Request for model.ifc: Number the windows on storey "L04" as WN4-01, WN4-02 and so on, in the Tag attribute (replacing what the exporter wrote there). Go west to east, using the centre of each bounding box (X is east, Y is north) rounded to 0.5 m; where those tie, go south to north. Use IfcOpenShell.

First a look at what the model holds.

```python
import ifcopenshell
import ifcopenshell.util.element
import ifcopenshell.util.placement

model = ifcopenshell.open("model.ifc")
print(model.schema)
storey = next(s for s in model.by_type("IfcBuildingStorey") if s.Name == "L04")
windows = [e for e in ifcopenshell.util.element.get_decomposition(storey) if e.is_a("IfcWindow")]
for e in sorted(windows, key=lambda e: e.id()):
    origin = ifcopenshell.util.placement.get_local_placement(e.ObjectPlacement)[:3, 3]
    print(e.id(), e.Tag, e.Name, origin.round(2) + 0.0, sep=" | ")
```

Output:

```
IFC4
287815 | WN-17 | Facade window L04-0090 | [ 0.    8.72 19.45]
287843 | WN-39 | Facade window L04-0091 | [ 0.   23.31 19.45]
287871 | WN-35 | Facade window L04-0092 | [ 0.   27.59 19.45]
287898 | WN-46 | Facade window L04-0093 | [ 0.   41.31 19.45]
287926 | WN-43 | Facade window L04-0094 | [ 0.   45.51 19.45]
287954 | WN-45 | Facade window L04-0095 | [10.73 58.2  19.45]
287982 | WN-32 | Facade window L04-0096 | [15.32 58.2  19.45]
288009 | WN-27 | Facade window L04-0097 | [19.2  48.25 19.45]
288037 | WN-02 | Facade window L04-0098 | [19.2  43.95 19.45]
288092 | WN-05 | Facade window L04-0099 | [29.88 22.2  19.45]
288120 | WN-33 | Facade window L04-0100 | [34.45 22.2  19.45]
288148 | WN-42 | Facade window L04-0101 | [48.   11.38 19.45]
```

```python
import ifcopenshell
import ifcopenshell.geom
import ifcopenshell.util.element
import ifcopenshell.util.shape

model = ifcopenshell.open("model.ifc")
settings = ifcopenshell.geom.settings()
settings.set("use-world-coords", True)


def centre(element):
    shape = ifcopenshell.geom.create_shape(settings, element)
    return ifcopenshell.util.shape.get_bbox_centroid(shape.geometry)


storey = next(s for s in model.by_type("IfcBuildingStorey") if s.Name == "L04")
windows = [e for e in ifcopenshell.util.element.get_decomposition(storey) if e.is_a("IfcWindow")]

# Insertion points can sit at a corner or the storey origin, so sort by the geometry (in metres).
centres = {e: centre(e) for e in windows}
windows.sort(key=lambda e: (round(centres[e][0] / 0.5), centres[e][1]))

for i, e in enumerate(windows, start=1):
    number = f"WN4-{i:02d}"
    e.Tag = number
    print(e.id(), number)

model.write("model_v2.ifc")
```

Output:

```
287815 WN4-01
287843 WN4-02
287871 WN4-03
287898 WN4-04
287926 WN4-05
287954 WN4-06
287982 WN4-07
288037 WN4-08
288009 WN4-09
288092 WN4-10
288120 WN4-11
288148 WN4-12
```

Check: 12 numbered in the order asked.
